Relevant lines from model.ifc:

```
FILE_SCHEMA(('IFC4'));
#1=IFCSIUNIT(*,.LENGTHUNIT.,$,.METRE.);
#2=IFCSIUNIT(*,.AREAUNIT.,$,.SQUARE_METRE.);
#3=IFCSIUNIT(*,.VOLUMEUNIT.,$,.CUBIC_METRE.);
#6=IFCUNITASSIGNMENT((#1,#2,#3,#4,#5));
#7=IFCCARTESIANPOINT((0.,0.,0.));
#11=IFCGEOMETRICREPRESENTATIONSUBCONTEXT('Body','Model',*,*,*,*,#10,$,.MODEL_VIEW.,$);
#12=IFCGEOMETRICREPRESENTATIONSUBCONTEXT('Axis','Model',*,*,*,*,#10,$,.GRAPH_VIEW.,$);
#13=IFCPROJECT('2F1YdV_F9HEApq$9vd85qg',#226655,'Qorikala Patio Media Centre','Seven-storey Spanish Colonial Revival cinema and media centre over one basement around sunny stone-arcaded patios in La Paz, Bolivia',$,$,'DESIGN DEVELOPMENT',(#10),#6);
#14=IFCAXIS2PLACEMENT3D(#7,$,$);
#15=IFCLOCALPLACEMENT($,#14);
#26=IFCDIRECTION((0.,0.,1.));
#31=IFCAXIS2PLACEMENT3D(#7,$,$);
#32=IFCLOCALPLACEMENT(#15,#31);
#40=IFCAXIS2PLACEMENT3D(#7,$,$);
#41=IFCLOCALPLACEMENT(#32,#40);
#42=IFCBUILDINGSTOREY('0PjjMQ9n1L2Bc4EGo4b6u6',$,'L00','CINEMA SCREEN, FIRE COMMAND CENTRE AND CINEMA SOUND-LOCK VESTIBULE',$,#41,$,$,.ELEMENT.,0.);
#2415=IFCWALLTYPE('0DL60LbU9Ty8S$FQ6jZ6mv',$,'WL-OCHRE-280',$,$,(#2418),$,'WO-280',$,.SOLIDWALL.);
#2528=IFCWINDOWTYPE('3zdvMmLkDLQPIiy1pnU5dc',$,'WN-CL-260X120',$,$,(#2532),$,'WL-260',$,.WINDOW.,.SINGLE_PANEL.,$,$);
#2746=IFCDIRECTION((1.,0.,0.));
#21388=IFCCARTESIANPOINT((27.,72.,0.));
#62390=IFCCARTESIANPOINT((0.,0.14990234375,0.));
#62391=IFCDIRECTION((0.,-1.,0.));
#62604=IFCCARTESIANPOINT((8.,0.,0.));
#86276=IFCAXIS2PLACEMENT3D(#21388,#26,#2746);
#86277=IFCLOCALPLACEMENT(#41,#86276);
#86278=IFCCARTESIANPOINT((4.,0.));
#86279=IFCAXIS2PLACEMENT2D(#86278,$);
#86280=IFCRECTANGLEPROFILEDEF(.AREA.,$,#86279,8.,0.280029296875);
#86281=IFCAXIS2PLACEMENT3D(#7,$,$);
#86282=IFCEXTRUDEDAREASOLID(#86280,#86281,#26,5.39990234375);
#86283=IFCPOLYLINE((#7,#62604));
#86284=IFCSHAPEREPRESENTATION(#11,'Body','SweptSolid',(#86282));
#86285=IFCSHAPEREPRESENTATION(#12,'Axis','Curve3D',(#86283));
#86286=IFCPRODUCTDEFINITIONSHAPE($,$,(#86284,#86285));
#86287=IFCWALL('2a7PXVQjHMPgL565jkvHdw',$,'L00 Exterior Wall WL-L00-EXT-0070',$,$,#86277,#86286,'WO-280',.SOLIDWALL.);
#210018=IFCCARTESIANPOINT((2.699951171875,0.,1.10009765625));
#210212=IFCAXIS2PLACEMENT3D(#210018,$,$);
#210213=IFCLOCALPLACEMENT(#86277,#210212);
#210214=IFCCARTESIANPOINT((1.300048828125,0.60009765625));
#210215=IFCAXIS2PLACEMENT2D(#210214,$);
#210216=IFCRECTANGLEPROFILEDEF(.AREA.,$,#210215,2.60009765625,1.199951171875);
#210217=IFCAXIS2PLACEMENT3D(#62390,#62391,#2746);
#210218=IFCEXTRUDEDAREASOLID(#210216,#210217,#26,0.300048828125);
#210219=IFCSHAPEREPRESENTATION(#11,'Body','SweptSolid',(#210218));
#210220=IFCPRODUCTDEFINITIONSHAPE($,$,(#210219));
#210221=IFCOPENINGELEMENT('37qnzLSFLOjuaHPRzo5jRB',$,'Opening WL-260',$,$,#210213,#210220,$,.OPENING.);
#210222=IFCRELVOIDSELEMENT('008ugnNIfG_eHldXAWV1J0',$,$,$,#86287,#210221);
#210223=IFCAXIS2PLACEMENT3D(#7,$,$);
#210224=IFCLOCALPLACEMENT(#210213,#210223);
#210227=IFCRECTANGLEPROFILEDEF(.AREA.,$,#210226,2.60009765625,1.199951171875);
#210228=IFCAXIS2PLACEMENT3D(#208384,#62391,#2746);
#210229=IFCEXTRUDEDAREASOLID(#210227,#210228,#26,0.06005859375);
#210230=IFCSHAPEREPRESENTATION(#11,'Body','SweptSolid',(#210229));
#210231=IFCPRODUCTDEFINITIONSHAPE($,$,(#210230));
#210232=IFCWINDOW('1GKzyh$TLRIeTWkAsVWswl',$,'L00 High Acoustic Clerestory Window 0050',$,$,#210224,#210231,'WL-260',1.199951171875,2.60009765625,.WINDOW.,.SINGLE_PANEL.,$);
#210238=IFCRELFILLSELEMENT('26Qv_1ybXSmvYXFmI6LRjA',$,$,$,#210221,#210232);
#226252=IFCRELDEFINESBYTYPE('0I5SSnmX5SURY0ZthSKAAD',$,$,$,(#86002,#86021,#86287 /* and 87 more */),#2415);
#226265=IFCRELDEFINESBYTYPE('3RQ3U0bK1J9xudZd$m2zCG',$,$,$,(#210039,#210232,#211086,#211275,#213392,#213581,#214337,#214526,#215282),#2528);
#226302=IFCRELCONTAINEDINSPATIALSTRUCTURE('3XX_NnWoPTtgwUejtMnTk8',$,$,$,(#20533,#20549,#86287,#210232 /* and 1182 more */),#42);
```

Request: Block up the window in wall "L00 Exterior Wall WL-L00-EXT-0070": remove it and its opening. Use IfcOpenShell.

```python
import ifcopenshell
import ifcopenshell.api.feature
import ifcopenshell.api.root
import ifcopenshell.geom
import ifcopenshell.util.shape

model = ifcopenshell.open("model.ifc")
settings = ifcopenshell.geom.settings()


def volume(element):
    """Net volume in cubic metres, openings subtracted."""
    shape = ifcopenshell.geom.create_shape(settings, element)
    return ifcopenshell.util.shape.get_volume(shape.geometry)


window = model.by_id(210232)
opening = window.FillsVoids[0].RelatingOpeningElement
wall = opening.VoidsElements[0].RelatingBuildingElement
before = volume(wall)

ifcopenshell.api.root.remove_product(model, product=window)
ifcopenshell.api.feature.remove_feature(model, feature=opening)

after = volume(wall)

print(f"wall volume {before:.3f} -> {after:.3f} m3")

model.write("model_edited.ifc")
```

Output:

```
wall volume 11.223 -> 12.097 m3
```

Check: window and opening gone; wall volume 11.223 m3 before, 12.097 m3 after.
